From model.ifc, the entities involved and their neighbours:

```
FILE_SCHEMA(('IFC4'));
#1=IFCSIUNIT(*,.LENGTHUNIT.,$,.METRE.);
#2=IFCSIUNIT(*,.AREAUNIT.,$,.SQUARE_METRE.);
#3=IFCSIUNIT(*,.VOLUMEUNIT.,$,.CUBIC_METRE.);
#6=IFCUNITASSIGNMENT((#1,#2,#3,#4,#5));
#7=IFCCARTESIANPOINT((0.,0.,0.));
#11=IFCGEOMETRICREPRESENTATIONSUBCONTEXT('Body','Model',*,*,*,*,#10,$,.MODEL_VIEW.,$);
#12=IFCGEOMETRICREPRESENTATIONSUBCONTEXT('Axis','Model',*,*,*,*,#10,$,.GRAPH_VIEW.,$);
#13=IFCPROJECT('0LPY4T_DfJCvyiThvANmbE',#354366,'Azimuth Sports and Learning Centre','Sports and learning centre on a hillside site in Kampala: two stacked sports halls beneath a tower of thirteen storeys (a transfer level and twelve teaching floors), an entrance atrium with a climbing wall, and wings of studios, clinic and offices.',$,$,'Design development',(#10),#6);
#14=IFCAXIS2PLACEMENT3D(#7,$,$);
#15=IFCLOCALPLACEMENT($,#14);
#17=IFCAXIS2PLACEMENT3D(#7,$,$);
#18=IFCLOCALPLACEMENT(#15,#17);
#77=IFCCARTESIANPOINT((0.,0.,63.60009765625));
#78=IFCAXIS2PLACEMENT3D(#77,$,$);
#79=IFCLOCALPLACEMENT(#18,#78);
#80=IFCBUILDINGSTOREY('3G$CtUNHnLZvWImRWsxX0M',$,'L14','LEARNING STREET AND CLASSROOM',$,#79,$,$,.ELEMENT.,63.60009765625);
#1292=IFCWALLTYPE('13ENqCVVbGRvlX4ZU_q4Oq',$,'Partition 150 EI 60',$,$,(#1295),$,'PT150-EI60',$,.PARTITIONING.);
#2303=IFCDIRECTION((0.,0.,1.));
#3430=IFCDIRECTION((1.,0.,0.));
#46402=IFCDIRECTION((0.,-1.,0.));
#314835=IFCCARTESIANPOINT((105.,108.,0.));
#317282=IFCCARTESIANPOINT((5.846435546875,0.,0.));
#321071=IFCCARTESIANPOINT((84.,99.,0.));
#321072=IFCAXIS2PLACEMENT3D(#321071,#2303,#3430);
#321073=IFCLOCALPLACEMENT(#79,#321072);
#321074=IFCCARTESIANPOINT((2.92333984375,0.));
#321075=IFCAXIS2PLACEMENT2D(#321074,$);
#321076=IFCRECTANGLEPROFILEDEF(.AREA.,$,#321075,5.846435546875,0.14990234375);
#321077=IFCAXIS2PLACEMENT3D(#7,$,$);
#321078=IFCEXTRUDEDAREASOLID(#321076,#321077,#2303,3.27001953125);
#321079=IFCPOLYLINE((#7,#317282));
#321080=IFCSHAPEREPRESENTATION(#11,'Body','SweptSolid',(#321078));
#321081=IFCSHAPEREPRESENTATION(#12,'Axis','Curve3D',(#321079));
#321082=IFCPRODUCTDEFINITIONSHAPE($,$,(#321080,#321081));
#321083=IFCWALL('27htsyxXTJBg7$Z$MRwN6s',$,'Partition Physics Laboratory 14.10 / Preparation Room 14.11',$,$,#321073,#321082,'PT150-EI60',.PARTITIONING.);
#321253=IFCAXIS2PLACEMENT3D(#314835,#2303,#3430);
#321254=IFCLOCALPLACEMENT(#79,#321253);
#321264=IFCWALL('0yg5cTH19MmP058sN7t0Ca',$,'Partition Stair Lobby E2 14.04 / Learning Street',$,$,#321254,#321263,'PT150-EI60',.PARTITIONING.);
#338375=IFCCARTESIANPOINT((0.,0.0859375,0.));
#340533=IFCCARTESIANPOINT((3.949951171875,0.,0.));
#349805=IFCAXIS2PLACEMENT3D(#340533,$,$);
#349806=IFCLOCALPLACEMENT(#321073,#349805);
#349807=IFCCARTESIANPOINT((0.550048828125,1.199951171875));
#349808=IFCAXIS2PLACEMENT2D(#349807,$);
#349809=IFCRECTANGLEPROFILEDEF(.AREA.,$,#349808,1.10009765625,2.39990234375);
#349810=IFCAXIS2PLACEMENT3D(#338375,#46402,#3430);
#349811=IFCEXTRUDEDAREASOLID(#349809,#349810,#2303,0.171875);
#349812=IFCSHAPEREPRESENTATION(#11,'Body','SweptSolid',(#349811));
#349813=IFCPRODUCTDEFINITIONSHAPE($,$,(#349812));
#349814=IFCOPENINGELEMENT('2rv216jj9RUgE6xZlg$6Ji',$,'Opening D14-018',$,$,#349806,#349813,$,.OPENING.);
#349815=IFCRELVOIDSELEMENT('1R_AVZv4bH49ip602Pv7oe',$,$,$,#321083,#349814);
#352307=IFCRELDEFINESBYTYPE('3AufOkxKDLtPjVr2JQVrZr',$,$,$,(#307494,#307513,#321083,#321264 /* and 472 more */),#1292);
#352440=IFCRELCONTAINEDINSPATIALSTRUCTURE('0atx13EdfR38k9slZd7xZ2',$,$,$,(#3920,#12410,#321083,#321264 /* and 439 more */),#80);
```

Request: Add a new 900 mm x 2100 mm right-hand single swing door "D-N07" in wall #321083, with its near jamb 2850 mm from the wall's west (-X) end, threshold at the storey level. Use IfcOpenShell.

```python
import numpy as np
import ifcopenshell
import ifcopenshell.api.feature
import ifcopenshell.api.geometry
import ifcopenshell.api.root
import ifcopenshell.api.spatial
import ifcopenshell.geom
import ifcopenshell.util.element
import ifcopenshell.util.placement
import ifcopenshell.util.representation
import ifcopenshell.util.shape
import ifcopenshell.util.unit

model = ifcopenshell.open("model.ifc")
unit_scale = ifcopenshell.util.unit.calculate_unit_scale(model)
settings = ifcopenshell.geom.settings()


def volume(element):
    """Net volume in cubic metres, openings subtracted."""
    shape = ifcopenshell.geom.create_shape(settings, element)
    return ifcopenshell.util.shape.get_volume(shape.geometry)


wall = model.by_guid("27htsyxXTJBg7$Z$MRwN6s")
storey = ifcopenshell.util.element.get_container(wall, ifc_class="IfcBuildingStorey")
context = ifcopenshell.util.representation.get_context(model, "Model", "Body", "MODEL_VIEW")
before = volume(wall)

width, height, from_end, sill = 0.9, 2.1, 2.85, 0.0  # metres

# The wall runs along its own X axis, and the end named is its -X end.
wall_shape = ifcopenshell.geom.create_shape(settings, wall)
x, y, z = ifcopenshell.util.shape.get_vertices(wall_shape.geometry).T
start = x.min() + from_end
face, thickness = float(y.min()), float(y.max() - y.min())
wall_matrix = ifcopenshell.util.placement.get_local_placement(wall.ObjectPlacement)
level = ifcopenshell.util.placement.get_local_placement(storey.ObjectPlacement)[2, 3]


def in_wall(x, y):
    """Placement at x, y metres in the wall's axes, at sill height."""
    matrix = wall_matrix.copy()
    matrix[:, 3] = wall_matrix @ np.array([x / unit_scale, y / unit_scale, 0.0, 1.0])
    matrix[2, 3] = level + sill / unit_scale
    return matrix


# Opening: a box that overshoots both wall faces by 50 mm.
opening = ifcopenshell.api.root.create_entity(model, ifc_class="IfcOpeningElement", predefined_type="OPENING")
box = ifcopenshell.api.geometry.add_wall_representation(
    model, context=context, length=width, height=height, thickness=thickness + 0.1
)
ifcopenshell.api.geometry.assign_representation(model, product=opening, representation=box)
ifcopenshell.api.geometry.edit_object_placement(model, product=opening, matrix=in_wall(start, face - 0.05), is_si=False)
ifcopenshell.api.feature.add_feature(model, feature=opening, element=wall)

door = ifcopenshell.api.root.create_entity(model, ifc_class="IfcDoor", name="D-N07", predefined_type="DOOR")
door.OverallWidth, door.OverallHeight = width / unit_scale, height / unit_scale
door.OperationType = "SINGLE_SWING_RIGHT"
body = ifcopenshell.api.geometry.add_door_representation(
    model,
    context=context,
    overall_width=door.OverallWidth,
    overall_height=door.OverallHeight,
    operation_type="SINGLE_SWING_RIGHT",
    lining_properties={"LiningDepth": thickness / unit_scale, "ThresholdDepth": thickness / unit_scale},
)
ifcopenshell.api.geometry.assign_representation(model, product=door, representation=body)
ifcopenshell.api.spatial.assign_container(model, products=[door], relating_structure=storey)
ifcopenshell.api.feature.add_filling(model, opening=opening, element=door)

# The lining spans the wall, so the door starts at the wall face.
ifcopenshell.api.geometry.edit_object_placement(model, product=door, matrix=in_wall(start, face), is_si=False)

after = volume(wall)

print(f"wall volume {before:.3f} -> {after:.3f} m3")

model.write("model_edited.ifc")
```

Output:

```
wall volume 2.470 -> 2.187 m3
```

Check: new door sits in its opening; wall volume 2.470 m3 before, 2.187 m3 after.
